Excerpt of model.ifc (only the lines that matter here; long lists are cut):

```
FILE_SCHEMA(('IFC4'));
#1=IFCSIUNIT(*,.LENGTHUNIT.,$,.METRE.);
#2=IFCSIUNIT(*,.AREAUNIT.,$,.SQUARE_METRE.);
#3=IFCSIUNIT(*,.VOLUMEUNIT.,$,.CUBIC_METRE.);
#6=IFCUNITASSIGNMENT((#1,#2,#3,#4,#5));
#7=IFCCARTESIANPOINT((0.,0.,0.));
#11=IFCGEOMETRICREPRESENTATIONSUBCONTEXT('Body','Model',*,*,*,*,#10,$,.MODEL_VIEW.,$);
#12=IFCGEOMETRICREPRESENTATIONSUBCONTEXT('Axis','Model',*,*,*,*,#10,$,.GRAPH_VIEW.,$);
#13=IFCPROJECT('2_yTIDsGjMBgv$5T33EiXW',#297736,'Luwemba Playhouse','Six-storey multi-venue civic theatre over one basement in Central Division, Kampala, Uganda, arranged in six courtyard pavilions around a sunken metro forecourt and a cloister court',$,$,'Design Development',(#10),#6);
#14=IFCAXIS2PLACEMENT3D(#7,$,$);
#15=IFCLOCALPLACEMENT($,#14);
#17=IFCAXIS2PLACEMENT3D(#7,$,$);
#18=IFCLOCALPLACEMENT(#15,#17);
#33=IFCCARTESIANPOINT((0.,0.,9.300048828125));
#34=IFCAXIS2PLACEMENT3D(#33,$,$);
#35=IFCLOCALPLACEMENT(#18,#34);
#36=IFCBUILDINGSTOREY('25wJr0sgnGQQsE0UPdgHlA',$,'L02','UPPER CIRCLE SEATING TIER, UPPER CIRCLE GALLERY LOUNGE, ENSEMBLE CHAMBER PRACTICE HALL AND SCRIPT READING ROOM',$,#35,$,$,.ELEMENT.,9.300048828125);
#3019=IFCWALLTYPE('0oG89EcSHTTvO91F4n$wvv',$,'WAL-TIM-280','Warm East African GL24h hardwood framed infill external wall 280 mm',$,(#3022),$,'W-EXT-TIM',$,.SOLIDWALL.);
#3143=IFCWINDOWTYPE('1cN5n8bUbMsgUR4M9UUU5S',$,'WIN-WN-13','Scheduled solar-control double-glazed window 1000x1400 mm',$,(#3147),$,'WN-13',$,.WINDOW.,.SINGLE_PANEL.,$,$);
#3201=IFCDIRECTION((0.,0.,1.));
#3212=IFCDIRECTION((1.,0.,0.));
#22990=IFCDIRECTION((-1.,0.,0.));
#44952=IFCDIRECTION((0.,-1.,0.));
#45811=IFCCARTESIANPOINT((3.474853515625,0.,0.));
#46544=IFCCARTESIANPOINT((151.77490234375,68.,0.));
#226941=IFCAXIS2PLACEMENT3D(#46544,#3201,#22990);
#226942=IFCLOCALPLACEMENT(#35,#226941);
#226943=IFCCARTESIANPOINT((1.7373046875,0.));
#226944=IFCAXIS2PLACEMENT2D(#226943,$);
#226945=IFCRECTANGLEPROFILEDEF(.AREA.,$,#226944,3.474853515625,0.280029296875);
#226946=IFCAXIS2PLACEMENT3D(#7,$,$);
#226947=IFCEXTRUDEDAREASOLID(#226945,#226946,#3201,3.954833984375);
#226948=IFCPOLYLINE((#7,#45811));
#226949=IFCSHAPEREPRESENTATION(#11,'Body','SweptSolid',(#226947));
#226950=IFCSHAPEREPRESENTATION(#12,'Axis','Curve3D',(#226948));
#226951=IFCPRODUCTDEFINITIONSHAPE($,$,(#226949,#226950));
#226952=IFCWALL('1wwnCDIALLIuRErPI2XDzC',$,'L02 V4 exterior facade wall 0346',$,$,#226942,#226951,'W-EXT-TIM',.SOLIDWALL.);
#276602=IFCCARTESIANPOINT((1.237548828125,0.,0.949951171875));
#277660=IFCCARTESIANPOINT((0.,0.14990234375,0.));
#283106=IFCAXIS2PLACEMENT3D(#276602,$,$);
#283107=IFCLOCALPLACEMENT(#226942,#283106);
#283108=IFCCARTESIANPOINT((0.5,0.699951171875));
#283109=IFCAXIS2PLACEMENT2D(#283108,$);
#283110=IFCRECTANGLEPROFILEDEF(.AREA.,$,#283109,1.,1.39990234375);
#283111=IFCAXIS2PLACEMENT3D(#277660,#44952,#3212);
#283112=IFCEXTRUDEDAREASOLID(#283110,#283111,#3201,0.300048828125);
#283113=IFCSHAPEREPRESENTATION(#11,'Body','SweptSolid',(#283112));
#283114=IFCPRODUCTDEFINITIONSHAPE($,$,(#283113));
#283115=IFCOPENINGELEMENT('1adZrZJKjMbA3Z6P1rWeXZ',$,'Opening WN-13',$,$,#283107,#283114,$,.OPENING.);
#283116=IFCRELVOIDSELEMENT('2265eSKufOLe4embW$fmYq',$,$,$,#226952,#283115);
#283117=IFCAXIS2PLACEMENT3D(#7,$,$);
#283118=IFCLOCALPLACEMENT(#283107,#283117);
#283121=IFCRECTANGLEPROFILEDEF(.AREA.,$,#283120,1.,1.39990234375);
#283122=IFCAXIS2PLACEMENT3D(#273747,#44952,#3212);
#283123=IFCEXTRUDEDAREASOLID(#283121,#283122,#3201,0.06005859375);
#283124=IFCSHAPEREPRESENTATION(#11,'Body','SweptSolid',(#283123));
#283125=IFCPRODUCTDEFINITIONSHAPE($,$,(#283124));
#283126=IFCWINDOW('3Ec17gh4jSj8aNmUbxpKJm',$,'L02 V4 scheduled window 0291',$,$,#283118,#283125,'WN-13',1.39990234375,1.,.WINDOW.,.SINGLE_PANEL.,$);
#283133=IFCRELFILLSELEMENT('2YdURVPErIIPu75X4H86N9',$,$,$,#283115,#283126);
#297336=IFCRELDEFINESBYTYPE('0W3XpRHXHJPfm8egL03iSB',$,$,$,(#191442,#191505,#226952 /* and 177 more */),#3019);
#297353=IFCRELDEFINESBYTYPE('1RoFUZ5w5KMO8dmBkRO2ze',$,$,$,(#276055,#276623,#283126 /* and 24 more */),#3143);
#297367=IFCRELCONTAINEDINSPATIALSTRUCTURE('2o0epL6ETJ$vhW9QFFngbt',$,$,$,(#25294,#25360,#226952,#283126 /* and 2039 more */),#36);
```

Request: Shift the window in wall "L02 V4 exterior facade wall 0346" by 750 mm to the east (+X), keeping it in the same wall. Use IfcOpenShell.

```python
import ifcopenshell
import ifcopenshell.api.geometry
import ifcopenshell.util.placement
import ifcopenshell.util.unit

model = ifcopenshell.open("model.ifc")
unit_scale = ifcopenshell.util.unit.calculate_unit_scale(model)

window = model.by_guid("3Ec17gh4jSj8aNmUbxpKJm")
opening = window.FillsVoids[0].RelatingOpeningElement
wall = opening.VoidsElements[0].RelatingBuildingElement

wall_matrix = ifcopenshell.util.placement.get_local_placement(wall.ObjectPlacement)
shift = wall_matrix[:3, 0] * -0.75 / unit_scale
before = ifcopenshell.util.placement.get_local_placement(window.ObjectPlacement)[:3, 3].copy()

# The window is placed relative to its opening, so it follows when the opening moves.
matrix = ifcopenshell.util.placement.get_local_placement(opening.ObjectPlacement)
matrix[:3, 3] += shift
ifcopenshell.api.geometry.edit_object_placement(
    model, product=opening, matrix=matrix, is_si=False, should_transform_children=True
)

after = ifcopenshell.util.placement.get_local_placement(window.ObjectPlacement)[:3, 3]
print("window moved by", (after - before).round(3) + 0.0)

model.write("model_updated.ifc")
```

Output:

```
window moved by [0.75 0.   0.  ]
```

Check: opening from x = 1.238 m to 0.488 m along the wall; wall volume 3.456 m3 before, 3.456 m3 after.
